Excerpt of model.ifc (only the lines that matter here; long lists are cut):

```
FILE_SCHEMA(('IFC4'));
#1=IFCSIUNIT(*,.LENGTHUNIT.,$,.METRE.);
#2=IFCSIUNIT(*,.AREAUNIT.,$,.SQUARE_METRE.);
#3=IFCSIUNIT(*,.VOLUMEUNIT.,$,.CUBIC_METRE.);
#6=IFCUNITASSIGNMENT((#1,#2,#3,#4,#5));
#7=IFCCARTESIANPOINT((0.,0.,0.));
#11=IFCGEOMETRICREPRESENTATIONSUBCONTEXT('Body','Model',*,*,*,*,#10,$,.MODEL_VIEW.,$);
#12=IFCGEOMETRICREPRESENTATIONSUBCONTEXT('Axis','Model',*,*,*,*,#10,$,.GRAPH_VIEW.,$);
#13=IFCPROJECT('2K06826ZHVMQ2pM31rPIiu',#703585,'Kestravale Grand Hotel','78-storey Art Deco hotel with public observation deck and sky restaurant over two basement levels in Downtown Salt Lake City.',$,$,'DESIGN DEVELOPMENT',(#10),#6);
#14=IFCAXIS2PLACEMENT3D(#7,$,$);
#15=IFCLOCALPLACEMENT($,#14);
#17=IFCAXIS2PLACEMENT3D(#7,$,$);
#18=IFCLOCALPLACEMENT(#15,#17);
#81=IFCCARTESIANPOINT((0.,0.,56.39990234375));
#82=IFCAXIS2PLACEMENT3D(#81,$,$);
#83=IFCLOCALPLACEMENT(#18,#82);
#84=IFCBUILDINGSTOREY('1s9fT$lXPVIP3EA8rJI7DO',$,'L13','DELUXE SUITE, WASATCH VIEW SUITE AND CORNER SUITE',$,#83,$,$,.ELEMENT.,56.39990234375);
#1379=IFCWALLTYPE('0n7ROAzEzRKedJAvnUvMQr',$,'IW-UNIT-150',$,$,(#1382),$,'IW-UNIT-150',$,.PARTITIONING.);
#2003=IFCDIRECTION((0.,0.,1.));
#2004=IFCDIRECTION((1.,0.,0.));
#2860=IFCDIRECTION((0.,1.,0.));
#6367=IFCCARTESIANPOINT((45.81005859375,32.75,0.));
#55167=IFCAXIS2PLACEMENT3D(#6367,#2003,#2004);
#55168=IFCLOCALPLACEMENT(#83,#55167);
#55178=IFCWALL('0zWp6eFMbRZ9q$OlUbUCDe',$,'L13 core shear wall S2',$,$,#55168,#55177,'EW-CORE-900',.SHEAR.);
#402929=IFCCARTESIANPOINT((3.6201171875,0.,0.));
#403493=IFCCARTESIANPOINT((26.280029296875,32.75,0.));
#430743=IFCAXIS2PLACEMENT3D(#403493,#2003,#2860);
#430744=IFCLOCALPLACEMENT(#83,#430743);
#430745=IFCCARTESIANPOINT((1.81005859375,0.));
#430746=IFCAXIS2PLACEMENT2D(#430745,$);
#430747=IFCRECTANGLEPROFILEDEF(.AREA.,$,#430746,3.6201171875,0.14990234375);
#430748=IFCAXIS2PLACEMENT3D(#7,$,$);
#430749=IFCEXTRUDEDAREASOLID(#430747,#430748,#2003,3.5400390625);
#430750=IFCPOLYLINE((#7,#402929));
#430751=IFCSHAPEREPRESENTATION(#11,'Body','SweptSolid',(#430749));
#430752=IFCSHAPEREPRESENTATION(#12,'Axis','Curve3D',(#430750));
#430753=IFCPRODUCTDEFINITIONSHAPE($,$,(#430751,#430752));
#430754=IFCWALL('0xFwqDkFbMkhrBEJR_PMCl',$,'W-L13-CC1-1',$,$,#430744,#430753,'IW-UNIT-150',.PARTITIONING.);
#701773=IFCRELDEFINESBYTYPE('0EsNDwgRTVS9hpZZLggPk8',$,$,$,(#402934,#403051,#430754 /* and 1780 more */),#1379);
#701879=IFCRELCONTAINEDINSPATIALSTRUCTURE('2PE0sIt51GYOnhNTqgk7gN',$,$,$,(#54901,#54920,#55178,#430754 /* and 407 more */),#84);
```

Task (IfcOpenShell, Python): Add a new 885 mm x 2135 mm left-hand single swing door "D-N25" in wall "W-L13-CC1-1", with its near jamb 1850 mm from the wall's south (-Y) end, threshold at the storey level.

```python
import numpy as np
import ifcopenshell
import ifcopenshell.api.feature
import ifcopenshell.api.geometry
import ifcopenshell.api.root
import ifcopenshell.api.spatial
import ifcopenshell.geom
import ifcopenshell.util.element
import ifcopenshell.util.placement
import ifcopenshell.util.representation
import ifcopenshell.util.shape
import ifcopenshell.util.unit

model = ifcopenshell.open("model.ifc")
unit_scale = ifcopenshell.util.unit.calculate_unit_scale(model)
settings = ifcopenshell.geom.settings()


def volume(element):
    """Net volume in cubic metres, openings subtracted."""
    shape = ifcopenshell.geom.create_shape(settings, element)
    return ifcopenshell.util.shape.get_volume(shape.geometry)


wall = model.by_guid("0xFwqDkFbMkhrBEJR_PMCl")
storey = ifcopenshell.util.element.get_container(wall, ifc_class="IfcBuildingStorey")
context = ifcopenshell.util.representation.get_context(model, "Model", "Body", "MODEL_VIEW")
before = volume(wall)

width, height, from_end, sill = 0.885, 2.135, 1.85, 0.0  # metres

# The wall runs along its own X axis, and the end named is its -X end.
wall_shape = ifcopenshell.geom.create_shape(settings, wall)
x, y, z = ifcopenshell.util.shape.get_vertices(wall_shape.geometry).T
start = x.min() + from_end
face, thickness = float(y.min()), float(y.max() - y.min())
wall_matrix = ifcopenshell.util.placement.get_local_placement(wall.ObjectPlacement)
level = ifcopenshell.util.placement.get_local_placement(storey.ObjectPlacement)[2, 3]


def in_wall(x, y):
    """Placement at x, y metres in the wall's axes, at sill height."""
    matrix = wall_matrix.copy()
    matrix[:, 3] = wall_matrix @ np.array([x / unit_scale, y / unit_scale, 0.0, 1.0])
    matrix[2, 3] = level + sill / unit_scale
    return matrix


# Opening: a box that overshoots both wall faces by 50 mm.
opening = ifcopenshell.api.root.create_entity(model, ifc_class="IfcOpeningElement", predefined_type="OPENING")
box = ifcopenshell.api.geometry.add_wall_representation(
    model, context=context, length=width, height=height, thickness=thickness + 0.1
)
ifcopenshell.api.geometry.assign_representation(model, product=opening, representation=box)
ifcopenshell.api.geometry.edit_object_placement(model, product=opening, matrix=in_wall(start, face - 0.05), is_si=False)
ifcopenshell.api.feature.add_feature(model, feature=opening, element=wall)

door = ifcopenshell.api.root.create_entity(model, ifc_class="IfcDoor", name="D-N25", predefined_type="DOOR")
door.OverallWidth, door.OverallHeight = width / unit_scale, height / unit_scale
door.OperationType = "SINGLE_SWING_LEFT"
body = ifcopenshell.api.geometry.add_door_representation(
    model,
    context=context,
    overall_width=door.OverallWidth,
    overall_height=door.OverallHeight,
    operation_type="SINGLE_SWING_LEFT",
    lining_properties={"LiningDepth": thickness / unit_scale, "ThresholdDepth": thickness / unit_scale},
)
ifcopenshell.api.geometry.assign_representation(model, product=door, representation=body)
ifcopenshell.api.spatial.assign_container(model, products=[door], relating_structure=storey)
ifcopenshell.api.feature.add_filling(model, opening=opening, element=door)

# The lining spans the wall, so the door starts at the wall face.
ifcopenshell.api.geometry.edit_object_placement(model, product=door, matrix=in_wall(start, face), is_si=False)

after = volume(wall)

print(f"wall volume {before:.3f} -> {after:.3f} m3")

model.write("model_v2.ifc")
```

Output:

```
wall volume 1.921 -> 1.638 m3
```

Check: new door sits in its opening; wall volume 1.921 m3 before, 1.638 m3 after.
